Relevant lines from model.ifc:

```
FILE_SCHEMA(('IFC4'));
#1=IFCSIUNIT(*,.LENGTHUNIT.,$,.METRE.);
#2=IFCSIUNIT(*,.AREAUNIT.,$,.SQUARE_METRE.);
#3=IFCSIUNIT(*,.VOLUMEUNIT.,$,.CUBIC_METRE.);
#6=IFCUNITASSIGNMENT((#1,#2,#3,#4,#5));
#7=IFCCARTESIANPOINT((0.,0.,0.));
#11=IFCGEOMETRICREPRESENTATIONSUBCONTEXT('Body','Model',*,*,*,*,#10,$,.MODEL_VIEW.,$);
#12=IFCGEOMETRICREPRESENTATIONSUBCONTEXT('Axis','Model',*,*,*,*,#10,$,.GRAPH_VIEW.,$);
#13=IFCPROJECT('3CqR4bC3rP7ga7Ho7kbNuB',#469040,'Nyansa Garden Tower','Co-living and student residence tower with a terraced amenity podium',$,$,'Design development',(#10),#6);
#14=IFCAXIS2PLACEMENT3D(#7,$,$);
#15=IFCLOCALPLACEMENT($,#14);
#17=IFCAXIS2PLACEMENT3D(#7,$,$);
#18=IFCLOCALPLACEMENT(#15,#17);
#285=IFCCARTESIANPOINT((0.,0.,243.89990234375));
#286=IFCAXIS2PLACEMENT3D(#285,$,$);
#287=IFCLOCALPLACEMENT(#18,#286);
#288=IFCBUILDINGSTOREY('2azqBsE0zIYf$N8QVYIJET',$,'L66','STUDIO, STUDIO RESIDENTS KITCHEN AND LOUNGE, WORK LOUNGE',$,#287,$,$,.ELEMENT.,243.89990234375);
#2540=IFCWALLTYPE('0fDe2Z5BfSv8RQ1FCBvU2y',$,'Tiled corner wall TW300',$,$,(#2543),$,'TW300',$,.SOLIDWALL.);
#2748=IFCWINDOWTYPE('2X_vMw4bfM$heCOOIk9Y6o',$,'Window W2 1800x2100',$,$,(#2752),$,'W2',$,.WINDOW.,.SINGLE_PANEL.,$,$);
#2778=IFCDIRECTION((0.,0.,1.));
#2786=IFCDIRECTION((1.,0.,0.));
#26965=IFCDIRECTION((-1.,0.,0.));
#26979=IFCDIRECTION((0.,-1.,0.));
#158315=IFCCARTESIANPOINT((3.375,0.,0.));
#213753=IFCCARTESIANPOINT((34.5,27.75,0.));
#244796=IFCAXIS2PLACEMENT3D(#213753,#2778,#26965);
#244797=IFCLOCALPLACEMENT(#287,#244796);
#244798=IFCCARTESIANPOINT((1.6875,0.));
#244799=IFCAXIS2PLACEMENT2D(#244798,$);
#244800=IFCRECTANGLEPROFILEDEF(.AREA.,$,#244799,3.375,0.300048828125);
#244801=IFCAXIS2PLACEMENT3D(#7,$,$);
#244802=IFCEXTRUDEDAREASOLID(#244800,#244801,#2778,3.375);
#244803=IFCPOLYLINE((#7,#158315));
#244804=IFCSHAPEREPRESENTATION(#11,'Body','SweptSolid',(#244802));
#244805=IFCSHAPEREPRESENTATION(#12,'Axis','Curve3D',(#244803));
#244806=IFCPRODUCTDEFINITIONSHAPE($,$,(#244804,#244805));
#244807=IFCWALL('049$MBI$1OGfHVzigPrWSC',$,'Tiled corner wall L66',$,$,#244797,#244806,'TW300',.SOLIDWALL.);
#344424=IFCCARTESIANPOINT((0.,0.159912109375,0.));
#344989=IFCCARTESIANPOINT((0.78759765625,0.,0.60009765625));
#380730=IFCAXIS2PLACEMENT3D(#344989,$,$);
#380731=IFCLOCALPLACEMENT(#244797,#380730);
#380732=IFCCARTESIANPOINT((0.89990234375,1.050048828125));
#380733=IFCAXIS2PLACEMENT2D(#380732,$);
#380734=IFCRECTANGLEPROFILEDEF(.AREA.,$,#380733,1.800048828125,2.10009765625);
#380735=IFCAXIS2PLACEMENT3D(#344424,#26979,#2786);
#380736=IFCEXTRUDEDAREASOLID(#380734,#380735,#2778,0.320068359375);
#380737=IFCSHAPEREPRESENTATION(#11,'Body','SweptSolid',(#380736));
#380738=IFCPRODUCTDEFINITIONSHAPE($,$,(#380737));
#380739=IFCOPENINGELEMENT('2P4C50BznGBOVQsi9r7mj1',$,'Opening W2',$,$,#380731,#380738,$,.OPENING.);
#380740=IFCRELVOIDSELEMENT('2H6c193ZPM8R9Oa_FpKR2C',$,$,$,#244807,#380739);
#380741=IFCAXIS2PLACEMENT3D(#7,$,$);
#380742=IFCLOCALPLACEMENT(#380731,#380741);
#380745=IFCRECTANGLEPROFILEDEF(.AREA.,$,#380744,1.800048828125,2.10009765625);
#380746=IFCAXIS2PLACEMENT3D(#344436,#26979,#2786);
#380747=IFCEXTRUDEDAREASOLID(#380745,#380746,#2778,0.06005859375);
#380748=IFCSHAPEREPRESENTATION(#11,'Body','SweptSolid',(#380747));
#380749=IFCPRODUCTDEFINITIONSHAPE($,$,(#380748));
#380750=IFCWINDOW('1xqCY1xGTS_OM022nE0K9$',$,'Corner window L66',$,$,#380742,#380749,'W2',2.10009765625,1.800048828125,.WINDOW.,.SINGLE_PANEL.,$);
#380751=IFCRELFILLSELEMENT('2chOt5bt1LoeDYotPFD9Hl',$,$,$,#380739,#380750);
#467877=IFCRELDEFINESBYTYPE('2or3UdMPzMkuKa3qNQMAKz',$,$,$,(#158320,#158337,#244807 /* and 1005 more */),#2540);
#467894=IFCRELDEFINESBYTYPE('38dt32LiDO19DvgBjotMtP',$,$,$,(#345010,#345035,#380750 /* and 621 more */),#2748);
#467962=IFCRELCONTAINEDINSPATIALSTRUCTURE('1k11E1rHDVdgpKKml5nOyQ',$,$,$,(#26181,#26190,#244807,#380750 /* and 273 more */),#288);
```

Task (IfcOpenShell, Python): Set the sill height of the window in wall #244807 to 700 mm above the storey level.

```python
import numpy as np
import ifcopenshell
import ifcopenshell.api.geometry
import ifcopenshell.geom
import ifcopenshell.util.element
import ifcopenshell.util.placement
import ifcopenshell.util.shape
import ifcopenshell.util.unit

model = ifcopenshell.open("model.ifc")
unit_scale = ifcopenshell.util.unit.calculate_unit_scale(model)

window = model.by_id(380750)
opening = window.FillsVoids[0].RelatingOpeningElement
storey = ifcopenshell.util.element.get_container(window, ifc_class="IfcBuildingStorey")
level = ifcopenshell.util.placement.get_local_placement(storey.ObjectPlacement)[2, 3]

# The opening's origin need not be at the sill, so measure its lowest point.
shape = ifcopenshell.geom.create_shape(ifcopenshell.geom.settings(), opening)
bottom = ifcopenshell.util.shape.get_shape_bottom_elevation(shape, shape.geometry) / unit_scale
dz = level + 0.7 / unit_scale - bottom

shift = np.array([0.0, 0.0, dz])
# The window is placed relative to its opening, so it follows when the opening moves.
matrix = ifcopenshell.util.placement.get_local_placement(opening.ObjectPlacement)
matrix[:3, 3] += shift
ifcopenshell.api.geometry.edit_object_placement(
    model, product=opening, matrix=matrix, is_si=False, should_transform_children=True
)

print(f"moved by {dz * unit_scale:+.3f} m")

model.write("model_rev.ifc")
```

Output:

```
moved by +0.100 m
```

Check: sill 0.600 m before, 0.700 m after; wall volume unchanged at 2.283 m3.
